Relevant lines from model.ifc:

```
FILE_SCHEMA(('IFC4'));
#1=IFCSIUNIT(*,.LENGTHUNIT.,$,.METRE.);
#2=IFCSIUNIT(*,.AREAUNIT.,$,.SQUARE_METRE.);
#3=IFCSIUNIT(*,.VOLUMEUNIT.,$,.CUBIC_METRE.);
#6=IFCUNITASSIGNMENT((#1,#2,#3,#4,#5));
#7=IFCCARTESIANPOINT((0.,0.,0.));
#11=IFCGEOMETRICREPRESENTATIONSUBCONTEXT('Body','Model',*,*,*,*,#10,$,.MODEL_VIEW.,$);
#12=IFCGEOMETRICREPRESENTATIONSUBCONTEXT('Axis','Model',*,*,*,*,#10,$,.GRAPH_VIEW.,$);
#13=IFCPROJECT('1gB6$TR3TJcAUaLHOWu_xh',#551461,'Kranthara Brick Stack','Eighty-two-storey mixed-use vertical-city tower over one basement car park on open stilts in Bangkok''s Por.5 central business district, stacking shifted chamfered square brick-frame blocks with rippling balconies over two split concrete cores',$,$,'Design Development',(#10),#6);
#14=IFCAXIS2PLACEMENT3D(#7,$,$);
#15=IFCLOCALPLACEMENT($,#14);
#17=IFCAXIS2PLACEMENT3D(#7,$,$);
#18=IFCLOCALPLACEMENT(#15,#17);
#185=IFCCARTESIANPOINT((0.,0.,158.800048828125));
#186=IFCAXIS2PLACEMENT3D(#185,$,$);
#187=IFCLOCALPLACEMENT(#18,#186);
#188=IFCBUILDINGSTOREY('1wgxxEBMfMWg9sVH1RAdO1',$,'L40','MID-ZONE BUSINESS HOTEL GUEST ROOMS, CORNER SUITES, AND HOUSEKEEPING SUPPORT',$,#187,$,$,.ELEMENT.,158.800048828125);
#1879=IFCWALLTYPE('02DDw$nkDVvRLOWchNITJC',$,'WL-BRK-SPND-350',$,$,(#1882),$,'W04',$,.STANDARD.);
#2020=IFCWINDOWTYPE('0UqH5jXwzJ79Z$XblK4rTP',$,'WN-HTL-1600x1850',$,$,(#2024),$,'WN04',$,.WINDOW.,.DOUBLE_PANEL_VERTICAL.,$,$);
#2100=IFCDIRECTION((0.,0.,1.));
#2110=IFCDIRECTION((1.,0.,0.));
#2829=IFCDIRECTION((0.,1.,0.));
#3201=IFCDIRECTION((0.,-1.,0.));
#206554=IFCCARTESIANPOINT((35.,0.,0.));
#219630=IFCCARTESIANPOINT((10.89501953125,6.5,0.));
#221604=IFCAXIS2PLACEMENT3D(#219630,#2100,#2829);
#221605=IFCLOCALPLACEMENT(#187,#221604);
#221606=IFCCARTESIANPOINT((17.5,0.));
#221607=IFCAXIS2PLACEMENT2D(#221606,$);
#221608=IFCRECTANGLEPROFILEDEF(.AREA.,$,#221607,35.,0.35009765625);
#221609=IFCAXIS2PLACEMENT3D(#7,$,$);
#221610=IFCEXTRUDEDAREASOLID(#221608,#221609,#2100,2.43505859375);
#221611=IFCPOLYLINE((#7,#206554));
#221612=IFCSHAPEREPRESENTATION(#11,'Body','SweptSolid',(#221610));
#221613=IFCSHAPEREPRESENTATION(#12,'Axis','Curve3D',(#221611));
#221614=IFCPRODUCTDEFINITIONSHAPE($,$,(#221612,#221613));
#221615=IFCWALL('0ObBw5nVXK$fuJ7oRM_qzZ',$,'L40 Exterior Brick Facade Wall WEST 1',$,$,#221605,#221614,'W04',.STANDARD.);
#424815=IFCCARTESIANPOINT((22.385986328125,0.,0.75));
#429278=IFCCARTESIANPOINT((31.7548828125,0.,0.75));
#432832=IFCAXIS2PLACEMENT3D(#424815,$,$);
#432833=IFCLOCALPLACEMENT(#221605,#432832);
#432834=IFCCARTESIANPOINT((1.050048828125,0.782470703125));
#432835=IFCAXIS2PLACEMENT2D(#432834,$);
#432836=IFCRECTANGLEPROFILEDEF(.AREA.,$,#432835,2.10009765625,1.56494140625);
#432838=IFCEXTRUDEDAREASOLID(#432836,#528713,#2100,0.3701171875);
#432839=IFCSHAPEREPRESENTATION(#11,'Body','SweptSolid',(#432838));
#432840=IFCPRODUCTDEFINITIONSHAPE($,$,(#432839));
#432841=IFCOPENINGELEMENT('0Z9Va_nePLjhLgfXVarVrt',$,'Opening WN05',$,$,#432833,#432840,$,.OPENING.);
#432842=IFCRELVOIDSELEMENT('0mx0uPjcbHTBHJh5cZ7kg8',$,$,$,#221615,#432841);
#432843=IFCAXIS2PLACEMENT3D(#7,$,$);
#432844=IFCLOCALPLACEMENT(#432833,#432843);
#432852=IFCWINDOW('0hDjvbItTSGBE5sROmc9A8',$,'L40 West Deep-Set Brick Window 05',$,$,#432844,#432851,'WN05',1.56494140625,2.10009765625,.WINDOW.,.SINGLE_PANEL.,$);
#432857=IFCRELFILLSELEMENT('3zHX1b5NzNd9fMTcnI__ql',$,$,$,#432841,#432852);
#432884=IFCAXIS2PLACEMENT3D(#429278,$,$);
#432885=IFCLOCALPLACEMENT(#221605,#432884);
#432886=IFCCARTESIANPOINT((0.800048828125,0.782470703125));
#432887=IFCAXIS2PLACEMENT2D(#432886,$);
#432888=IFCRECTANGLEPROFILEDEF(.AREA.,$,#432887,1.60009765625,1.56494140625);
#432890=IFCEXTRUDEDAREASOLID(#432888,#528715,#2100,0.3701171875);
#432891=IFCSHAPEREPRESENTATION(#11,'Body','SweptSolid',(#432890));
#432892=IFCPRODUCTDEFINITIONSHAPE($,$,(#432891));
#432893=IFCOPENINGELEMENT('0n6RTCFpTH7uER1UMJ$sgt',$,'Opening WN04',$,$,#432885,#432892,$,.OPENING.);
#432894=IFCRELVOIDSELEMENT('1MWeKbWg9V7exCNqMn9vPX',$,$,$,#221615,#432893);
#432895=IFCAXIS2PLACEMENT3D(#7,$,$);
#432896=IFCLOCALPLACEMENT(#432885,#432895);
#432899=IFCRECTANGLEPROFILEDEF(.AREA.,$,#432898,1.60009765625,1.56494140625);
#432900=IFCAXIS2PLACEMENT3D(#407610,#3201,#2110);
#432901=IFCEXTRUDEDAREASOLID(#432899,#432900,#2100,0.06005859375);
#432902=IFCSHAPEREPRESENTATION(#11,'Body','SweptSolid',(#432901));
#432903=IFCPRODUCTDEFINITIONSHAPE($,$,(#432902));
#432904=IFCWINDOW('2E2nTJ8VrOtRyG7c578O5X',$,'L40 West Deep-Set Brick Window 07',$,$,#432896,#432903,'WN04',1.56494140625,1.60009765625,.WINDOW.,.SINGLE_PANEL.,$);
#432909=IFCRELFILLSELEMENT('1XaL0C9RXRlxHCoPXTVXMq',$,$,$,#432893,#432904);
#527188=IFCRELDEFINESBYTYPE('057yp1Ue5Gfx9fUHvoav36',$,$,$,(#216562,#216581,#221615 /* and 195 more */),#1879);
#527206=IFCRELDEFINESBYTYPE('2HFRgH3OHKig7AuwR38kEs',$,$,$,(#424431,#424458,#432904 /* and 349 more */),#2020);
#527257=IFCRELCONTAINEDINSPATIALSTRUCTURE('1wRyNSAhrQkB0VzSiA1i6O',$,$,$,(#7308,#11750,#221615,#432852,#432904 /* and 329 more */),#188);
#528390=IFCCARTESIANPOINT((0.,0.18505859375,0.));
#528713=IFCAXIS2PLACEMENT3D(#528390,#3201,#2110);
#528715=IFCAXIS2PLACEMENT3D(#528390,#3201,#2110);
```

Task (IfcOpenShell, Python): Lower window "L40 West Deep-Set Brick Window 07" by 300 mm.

```python
import numpy as np
import ifcopenshell
import ifcopenshell.api.geometry
import ifcopenshell.util.placement
import ifcopenshell.util.unit

model = ifcopenshell.open("model.ifc")
unit_scale = ifcopenshell.util.unit.calculate_unit_scale(model)

window = model.by_guid("2E2nTJ8VrOtRyG7c578O5X")
opening = window.FillsVoids[0].RelatingOpeningElement
dz = -0.3

shift = np.array([0.0, 0.0, dz])
# The window is placed relative to its opening, so it follows when the opening moves.
matrix = ifcopenshell.util.placement.get_local_placement(opening.ObjectPlacement)
matrix[:3, 3] += shift
ifcopenshell.api.geometry.edit_object_placement(
    model, product=opening, matrix=matrix, is_si=False, should_transform_children=True
)

print(f"moved by {dz * unit_scale:+.3f} m")

model.write("model_edited.ifc")
```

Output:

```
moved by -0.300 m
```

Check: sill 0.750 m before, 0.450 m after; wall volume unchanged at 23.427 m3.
